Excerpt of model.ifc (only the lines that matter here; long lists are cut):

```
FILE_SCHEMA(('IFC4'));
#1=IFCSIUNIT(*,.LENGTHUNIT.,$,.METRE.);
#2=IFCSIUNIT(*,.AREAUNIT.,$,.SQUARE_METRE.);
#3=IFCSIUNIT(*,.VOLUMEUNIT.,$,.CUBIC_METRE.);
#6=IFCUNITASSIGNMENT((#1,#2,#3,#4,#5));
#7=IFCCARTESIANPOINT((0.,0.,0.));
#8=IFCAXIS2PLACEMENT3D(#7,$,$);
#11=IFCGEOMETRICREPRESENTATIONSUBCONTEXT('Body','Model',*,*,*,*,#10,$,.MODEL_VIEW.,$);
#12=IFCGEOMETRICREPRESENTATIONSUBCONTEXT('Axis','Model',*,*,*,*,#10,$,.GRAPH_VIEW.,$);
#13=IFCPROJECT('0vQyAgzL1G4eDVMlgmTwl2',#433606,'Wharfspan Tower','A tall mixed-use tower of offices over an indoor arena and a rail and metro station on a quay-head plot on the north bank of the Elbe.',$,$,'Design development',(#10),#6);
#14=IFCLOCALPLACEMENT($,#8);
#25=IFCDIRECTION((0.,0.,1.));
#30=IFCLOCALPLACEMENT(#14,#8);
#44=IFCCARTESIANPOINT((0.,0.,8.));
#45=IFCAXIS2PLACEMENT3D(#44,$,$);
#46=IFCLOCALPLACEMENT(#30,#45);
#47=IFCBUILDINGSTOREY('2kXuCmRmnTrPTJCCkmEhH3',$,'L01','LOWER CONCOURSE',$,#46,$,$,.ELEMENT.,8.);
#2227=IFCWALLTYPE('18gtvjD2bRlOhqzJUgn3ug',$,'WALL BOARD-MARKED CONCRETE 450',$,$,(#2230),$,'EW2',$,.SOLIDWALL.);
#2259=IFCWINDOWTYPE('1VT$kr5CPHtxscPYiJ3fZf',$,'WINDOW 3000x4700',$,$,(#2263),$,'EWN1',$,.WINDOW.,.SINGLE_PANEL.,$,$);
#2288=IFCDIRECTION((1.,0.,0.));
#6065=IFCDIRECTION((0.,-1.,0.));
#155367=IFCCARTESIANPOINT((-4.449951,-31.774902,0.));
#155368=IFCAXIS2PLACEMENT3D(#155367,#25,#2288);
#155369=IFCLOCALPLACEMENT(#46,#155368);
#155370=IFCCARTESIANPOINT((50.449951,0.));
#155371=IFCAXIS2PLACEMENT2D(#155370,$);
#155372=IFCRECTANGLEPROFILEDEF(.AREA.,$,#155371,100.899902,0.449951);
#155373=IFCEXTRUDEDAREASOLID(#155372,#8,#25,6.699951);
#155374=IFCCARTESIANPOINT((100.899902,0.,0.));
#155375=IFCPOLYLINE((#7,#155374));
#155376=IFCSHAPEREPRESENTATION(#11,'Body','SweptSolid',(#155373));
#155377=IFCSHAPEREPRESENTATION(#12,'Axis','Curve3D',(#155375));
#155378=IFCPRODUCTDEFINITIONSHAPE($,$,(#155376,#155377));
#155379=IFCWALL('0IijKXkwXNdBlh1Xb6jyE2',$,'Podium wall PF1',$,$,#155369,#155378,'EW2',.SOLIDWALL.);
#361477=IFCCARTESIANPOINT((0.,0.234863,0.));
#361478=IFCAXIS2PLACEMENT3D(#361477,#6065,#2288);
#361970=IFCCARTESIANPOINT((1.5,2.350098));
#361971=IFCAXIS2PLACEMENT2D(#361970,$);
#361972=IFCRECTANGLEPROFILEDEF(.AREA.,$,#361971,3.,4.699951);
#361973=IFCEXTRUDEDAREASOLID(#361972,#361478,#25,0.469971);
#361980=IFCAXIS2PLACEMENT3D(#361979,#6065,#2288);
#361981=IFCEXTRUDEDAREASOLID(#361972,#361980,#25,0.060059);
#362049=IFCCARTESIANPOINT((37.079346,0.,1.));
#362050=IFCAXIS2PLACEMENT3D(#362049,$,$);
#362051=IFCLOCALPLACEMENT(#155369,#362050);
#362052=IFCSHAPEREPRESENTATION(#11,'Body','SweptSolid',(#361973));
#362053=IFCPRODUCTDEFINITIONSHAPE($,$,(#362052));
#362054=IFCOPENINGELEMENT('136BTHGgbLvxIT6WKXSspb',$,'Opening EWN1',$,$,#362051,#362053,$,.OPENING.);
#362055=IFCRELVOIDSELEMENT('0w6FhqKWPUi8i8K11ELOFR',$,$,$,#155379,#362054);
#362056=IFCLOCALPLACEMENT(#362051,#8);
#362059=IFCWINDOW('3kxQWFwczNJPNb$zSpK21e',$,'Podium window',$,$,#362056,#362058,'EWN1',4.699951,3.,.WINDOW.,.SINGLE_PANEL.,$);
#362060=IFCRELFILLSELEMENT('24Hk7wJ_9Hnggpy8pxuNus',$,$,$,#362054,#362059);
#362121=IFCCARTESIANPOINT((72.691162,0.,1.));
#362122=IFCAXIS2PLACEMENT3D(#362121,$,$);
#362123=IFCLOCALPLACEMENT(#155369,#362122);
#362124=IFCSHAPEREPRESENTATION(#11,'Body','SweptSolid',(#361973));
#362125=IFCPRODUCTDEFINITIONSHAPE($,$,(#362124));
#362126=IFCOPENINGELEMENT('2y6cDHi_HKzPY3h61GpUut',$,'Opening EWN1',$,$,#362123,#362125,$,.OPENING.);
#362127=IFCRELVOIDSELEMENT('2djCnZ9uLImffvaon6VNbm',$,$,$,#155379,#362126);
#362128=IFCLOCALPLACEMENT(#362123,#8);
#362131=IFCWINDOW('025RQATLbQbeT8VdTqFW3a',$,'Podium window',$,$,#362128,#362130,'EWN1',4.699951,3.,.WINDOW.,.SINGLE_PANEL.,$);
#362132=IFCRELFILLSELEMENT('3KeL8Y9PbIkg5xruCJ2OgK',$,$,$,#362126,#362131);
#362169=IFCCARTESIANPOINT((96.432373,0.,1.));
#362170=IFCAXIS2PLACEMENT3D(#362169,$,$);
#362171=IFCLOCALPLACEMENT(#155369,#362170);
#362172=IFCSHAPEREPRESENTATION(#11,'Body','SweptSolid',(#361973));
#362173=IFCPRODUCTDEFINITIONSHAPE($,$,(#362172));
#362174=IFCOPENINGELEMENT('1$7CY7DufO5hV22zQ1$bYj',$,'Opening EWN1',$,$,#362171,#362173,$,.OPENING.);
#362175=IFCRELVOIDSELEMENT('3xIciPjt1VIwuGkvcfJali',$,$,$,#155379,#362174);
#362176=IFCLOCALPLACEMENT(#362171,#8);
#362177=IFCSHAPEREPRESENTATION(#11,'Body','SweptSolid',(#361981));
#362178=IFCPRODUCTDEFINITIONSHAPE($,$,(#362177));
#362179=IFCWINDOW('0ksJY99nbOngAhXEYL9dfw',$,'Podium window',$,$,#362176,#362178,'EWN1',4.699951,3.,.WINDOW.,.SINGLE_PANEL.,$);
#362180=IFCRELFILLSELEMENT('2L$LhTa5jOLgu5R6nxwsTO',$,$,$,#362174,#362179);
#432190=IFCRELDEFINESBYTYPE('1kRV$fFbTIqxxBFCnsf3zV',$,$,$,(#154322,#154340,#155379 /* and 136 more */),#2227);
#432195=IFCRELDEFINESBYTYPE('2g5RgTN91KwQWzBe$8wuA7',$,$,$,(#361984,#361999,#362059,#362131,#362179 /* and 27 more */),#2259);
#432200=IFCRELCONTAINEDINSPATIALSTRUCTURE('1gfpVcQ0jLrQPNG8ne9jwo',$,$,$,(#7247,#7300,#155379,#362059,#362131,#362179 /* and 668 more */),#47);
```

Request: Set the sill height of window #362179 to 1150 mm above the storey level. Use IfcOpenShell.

```python
import numpy as np
import ifcopenshell
import ifcopenshell.api.geometry
import ifcopenshell.geom
import ifcopenshell.util.element
import ifcopenshell.util.placement
import ifcopenshell.util.shape
import ifcopenshell.util.unit

model = ifcopenshell.open("model.ifc")
unit_scale = ifcopenshell.util.unit.calculate_unit_scale(model)

window = model.by_guid("0ksJY99nbOngAhXEYL9dfw")
opening = window.FillsVoids[0].RelatingOpeningElement
storey = ifcopenshell.util.element.get_container(window, ifc_class="IfcBuildingStorey")
level = ifcopenshell.util.placement.get_local_placement(storey.ObjectPlacement)[2, 3]

# The opening's origin need not be at the sill, so measure its lowest point.
shape = ifcopenshell.geom.create_shape(ifcopenshell.geom.settings(), opening)
bottom = ifcopenshell.util.shape.get_shape_bottom_elevation(shape, shape.geometry) / unit_scale
dz = level + 1.15 / unit_scale - bottom

shift = np.array([0.0, 0.0, dz])
# The window is placed relative to its opening, so it follows when the opening moves.
matrix = ifcopenshell.util.placement.get_local_placement(opening.ObjectPlacement)
matrix[:3, 3] += shift
ifcopenshell.api.geometry.edit_object_placement(
    model, product=opening, matrix=matrix, is_si=False, should_transform_children=True
)

print(f"moved by {dz * unit_scale:+.3f} m")

model.write("model-out.ifc")
```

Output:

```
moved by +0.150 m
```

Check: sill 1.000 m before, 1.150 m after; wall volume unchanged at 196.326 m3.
